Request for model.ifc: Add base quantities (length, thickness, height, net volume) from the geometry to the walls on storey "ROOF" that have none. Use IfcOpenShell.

First a look at what the model holds.

```python
import ifcopenshell
import ifcopenshell.util.element
import ifcopenshell.util.unit

model = ifcopenshell.open("model.ifc")
print(model.schema)
for unit_type in ("LENGTHUNIT", "AREAUNIT", "VOLUMEUNIT"):
    print(unit_type, ifcopenshell.util.unit.calculate_unit_scale(model, unit_type))
storey = next(s for s in model.by_type("IfcBuildingStorey") if s.Name == "ROOF")
walls = [e for e in ifcopenshell.util.element.get_decomposition(storey) if e.is_a("IfcWall")]
for e in sorted(walls, key=lambda e: e.id()):
    print(e.id(), e.is_a(), e.Name, list(ifcopenshell.util.element.get_psets(e, qtos_only=True)), sep=" | ")
```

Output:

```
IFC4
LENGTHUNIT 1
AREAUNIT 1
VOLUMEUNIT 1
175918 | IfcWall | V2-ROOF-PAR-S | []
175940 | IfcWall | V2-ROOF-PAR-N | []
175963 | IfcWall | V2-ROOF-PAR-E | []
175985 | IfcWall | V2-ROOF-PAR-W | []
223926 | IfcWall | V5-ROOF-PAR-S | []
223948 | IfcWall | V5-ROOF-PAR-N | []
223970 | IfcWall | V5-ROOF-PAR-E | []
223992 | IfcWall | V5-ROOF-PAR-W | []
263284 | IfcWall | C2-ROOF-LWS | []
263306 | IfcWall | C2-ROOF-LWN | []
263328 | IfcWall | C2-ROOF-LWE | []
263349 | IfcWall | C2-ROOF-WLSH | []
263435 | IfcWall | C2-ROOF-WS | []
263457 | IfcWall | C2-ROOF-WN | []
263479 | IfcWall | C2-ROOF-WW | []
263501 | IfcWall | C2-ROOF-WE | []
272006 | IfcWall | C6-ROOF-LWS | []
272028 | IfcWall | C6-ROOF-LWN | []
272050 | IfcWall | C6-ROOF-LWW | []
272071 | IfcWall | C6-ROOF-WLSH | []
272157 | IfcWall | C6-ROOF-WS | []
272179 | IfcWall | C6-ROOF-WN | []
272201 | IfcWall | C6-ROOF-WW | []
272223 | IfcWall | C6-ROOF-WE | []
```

```python
import ifcopenshell
import ifcopenshell.api.pset
import ifcopenshell.geom
import ifcopenshell.util.element
import ifcopenshell.util.shape
import ifcopenshell.util.unit

model = ifcopenshell.open("model.ifc")
unit_scale = ifcopenshell.util.unit.calculate_unit_scale(model)
volume_scale = ifcopenshell.util.unit.calculate_unit_scale(model, "VOLUMEUNIT")
settings = ifcopenshell.geom.settings()

storey = next(s for s in model.by_type("IfcBuildingStorey") if s.Name == "ROOF")
walls = [e for e in ifcopenshell.util.element.get_decomposition(storey) if e.is_a("IfcWall")]

for e in sorted(walls, key=lambda e: e.id()):
    if ifcopenshell.util.element.get_psets(e, qtos_only=True, should_inherit=False):
        continue
    # Geometry comes back in metres, in the element's own axes.
    shape = ifcopenshell.geom.create_shape(settings, e)
    values = {
        "Length": ifcopenshell.util.shape.get_x(shape.geometry) / unit_scale,
        "Width": ifcopenshell.util.shape.get_y(shape.geometry) / unit_scale,
        "Height": ifcopenshell.util.shape.get_z(shape.geometry) / unit_scale,
        "NetVolume": ifcopenshell.util.shape.get_volume(shape.geometry) / volume_scale,
    }
    qto = ifcopenshell.api.pset.add_qto(model, product=e, name="Qto_WallBaseQuantities")
    ifcopenshell.api.pset.edit_qto(model, qto=qto, properties=values)
    print(e.id(), {k: round(v, 3) for k, v in values.items()})

model.write("model_rev.ifc")
```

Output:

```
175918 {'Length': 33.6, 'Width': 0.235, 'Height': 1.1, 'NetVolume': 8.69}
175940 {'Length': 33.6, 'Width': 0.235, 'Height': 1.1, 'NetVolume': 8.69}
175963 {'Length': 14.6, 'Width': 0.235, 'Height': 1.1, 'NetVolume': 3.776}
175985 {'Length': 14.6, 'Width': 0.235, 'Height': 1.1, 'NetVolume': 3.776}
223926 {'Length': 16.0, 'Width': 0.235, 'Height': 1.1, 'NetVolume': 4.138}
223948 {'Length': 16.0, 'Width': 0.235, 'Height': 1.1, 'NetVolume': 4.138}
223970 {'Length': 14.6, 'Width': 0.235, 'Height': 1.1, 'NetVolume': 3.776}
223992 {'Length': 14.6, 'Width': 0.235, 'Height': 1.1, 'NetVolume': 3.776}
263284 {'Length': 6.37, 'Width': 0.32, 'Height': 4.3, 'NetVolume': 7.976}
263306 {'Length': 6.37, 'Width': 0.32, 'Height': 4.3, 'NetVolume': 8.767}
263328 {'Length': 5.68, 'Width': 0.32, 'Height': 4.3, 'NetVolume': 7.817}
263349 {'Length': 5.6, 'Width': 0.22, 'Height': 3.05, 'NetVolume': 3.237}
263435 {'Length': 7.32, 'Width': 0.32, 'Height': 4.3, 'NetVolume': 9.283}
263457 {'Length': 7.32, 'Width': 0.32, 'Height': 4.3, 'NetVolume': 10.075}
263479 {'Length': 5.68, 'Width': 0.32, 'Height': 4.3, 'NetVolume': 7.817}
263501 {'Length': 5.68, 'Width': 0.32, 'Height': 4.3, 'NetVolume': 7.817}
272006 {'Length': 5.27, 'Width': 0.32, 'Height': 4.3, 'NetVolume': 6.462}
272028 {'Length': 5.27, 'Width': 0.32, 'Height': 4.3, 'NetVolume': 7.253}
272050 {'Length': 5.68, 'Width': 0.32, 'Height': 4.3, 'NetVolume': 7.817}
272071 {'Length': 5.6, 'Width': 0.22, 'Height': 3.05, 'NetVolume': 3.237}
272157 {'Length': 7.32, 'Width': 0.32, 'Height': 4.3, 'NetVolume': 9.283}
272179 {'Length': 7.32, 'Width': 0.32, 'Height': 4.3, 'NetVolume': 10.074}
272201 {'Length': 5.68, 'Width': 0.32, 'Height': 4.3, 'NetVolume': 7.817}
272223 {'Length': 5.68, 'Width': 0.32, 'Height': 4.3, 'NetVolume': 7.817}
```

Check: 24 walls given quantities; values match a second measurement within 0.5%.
